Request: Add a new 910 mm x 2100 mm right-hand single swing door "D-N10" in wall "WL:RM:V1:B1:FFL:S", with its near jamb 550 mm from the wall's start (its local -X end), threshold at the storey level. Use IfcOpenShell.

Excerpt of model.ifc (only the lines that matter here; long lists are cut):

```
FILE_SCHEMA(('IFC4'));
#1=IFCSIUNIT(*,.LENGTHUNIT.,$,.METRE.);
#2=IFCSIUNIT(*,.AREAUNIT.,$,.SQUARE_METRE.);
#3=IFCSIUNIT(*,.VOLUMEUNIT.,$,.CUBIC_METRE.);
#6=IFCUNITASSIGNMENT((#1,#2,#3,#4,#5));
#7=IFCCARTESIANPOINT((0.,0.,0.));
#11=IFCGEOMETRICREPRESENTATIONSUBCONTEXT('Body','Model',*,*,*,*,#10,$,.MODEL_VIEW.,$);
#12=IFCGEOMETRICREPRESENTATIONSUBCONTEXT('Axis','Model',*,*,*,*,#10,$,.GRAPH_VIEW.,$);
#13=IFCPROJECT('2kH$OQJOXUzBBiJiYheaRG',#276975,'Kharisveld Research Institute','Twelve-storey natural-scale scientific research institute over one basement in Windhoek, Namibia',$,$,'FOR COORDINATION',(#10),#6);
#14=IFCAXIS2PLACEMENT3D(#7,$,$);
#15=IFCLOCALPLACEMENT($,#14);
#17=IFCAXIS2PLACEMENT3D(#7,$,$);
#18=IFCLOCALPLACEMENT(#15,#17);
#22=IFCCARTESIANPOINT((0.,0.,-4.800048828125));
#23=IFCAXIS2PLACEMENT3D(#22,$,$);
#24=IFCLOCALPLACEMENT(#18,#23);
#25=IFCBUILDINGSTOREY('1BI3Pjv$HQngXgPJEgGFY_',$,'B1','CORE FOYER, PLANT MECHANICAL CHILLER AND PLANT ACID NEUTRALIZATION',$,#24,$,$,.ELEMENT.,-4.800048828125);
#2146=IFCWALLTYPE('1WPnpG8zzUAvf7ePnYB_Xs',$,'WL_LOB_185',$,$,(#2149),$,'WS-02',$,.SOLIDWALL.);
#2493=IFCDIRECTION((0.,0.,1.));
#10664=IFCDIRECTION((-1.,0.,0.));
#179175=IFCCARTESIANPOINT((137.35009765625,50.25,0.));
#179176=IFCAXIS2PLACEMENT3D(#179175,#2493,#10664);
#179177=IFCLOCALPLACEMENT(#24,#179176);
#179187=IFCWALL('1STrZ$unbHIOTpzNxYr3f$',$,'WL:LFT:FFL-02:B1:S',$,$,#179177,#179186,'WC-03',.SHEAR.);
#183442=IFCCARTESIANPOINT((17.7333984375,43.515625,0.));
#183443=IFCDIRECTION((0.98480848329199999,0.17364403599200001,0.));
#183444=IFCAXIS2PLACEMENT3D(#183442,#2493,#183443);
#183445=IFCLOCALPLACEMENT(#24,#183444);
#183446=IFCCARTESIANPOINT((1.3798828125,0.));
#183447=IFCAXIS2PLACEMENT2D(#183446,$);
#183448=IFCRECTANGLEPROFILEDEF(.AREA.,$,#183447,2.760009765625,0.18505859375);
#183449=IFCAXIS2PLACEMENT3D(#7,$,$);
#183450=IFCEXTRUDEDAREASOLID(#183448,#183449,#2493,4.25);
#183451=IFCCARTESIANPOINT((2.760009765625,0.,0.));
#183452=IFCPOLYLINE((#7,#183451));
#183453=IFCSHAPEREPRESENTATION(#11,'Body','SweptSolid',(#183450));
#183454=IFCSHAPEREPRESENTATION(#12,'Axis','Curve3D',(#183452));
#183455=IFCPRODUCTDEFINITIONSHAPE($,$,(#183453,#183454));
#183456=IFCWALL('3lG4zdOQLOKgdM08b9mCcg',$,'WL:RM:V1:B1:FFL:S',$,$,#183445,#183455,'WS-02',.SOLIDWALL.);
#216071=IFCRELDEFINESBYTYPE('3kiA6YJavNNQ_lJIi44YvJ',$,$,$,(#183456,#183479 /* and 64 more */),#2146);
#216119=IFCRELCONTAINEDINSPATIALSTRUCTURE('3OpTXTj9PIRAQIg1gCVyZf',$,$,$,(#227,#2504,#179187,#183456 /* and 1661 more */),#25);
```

```python
import numpy as np
import ifcopenshell
import ifcopenshell.api.feature
import ifcopenshell.api.geometry
import ifcopenshell.api.root
import ifcopenshell.api.spatial
import ifcopenshell.geom
import ifcopenshell.util.element
import ifcopenshell.util.placement
import ifcopenshell.util.representation
import ifcopenshell.util.shape
import ifcopenshell.util.unit

model = ifcopenshell.open("model.ifc")
unit_scale = ifcopenshell.util.unit.calculate_unit_scale(model)
settings = ifcopenshell.geom.settings()


def volume(element):
    """Net volume in cubic metres, openings subtracted."""
    shape = ifcopenshell.geom.create_shape(settings, element)
    return ifcopenshell.util.shape.get_volume(shape.geometry)


wall = model.by_guid("3lG4zdOQLOKgdM08b9mCcg")
storey = ifcopenshell.util.element.get_container(wall, ifc_class="IfcBuildingStorey")
context = ifcopenshell.util.representation.get_context(model, "Model", "Body", "MODEL_VIEW")
before = volume(wall)

width, height, from_end, sill = 0.91, 2.1, 0.55, 0.0  # metres

# The wall runs along its own X axis, and the end named is its -X end.
wall_shape = ifcopenshell.geom.create_shape(settings, wall)
x, y, z = ifcopenshell.util.shape.get_vertices(wall_shape.geometry).T
start = x.min() + from_end
face, thickness = float(y.min()), float(y.max() - y.min())
wall_matrix = ifcopenshell.util.placement.get_local_placement(wall.ObjectPlacement)
level = ifcopenshell.util.placement.get_local_placement(storey.ObjectPlacement)[2, 3]


def in_wall(x, y):
    """Placement at x, y metres in the wall's axes, at sill height."""
    matrix = wall_matrix.copy()
    matrix[:, 3] = wall_matrix @ np.array([x / unit_scale, y / unit_scale, 0.0, 1.0])
    matrix[2, 3] = level + sill / unit_scale
    return matrix


# Opening: a box that overshoots both wall faces by 50 mm.
opening = ifcopenshell.api.root.create_entity(model, ifc_class="IfcOpeningElement", predefined_type="OPENING")
box = ifcopenshell.api.geometry.add_wall_representation(
    model, context=context, length=width, height=height, thickness=thickness + 0.1
)
ifcopenshell.api.geometry.assign_representation(model, product=opening, representation=box)
ifcopenshell.api.geometry.edit_object_placement(model, product=opening, matrix=in_wall(start, face - 0.05), is_si=False)
ifcopenshell.api.feature.add_feature(model, feature=opening, element=wall)

door = ifcopenshell.api.root.create_entity(model, ifc_class="IfcDoor", name="D-N10", predefined_type="DOOR")
door.OverallWidth, door.OverallHeight = width / unit_scale, height / unit_scale
door.OperationType = "SINGLE_SWING_RIGHT"
body = ifcopenshell.api.geometry.add_door_representation(
    model,
    context=context,
    overall_width=door.OverallWidth,
    overall_height=door.OverallHeight,
    operation_type="SINGLE_SWING_RIGHT",
    lining_properties={"LiningDepth": thickness / unit_scale, "ThresholdDepth": thickness / unit_scale},
)
ifcopenshell.api.geometry.assign_representation(model, product=door, representation=body)
ifcopenshell.api.spatial.assign_container(model, products=[door], relating_structure=storey)
ifcopenshell.api.feature.add_filling(model, opening=opening, element=door)

# The lining spans the wall, so the door starts at the wall face.
ifcopenshell.api.geometry.edit_object_placement(model, product=door, matrix=in_wall(start, face), is_si=False)

after = volume(wall)

print(f"wall volume {before:.3f} -> {after:.3f} m3")

model.write("model_v2.ifc")
```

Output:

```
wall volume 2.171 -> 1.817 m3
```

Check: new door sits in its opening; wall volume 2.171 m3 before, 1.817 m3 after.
